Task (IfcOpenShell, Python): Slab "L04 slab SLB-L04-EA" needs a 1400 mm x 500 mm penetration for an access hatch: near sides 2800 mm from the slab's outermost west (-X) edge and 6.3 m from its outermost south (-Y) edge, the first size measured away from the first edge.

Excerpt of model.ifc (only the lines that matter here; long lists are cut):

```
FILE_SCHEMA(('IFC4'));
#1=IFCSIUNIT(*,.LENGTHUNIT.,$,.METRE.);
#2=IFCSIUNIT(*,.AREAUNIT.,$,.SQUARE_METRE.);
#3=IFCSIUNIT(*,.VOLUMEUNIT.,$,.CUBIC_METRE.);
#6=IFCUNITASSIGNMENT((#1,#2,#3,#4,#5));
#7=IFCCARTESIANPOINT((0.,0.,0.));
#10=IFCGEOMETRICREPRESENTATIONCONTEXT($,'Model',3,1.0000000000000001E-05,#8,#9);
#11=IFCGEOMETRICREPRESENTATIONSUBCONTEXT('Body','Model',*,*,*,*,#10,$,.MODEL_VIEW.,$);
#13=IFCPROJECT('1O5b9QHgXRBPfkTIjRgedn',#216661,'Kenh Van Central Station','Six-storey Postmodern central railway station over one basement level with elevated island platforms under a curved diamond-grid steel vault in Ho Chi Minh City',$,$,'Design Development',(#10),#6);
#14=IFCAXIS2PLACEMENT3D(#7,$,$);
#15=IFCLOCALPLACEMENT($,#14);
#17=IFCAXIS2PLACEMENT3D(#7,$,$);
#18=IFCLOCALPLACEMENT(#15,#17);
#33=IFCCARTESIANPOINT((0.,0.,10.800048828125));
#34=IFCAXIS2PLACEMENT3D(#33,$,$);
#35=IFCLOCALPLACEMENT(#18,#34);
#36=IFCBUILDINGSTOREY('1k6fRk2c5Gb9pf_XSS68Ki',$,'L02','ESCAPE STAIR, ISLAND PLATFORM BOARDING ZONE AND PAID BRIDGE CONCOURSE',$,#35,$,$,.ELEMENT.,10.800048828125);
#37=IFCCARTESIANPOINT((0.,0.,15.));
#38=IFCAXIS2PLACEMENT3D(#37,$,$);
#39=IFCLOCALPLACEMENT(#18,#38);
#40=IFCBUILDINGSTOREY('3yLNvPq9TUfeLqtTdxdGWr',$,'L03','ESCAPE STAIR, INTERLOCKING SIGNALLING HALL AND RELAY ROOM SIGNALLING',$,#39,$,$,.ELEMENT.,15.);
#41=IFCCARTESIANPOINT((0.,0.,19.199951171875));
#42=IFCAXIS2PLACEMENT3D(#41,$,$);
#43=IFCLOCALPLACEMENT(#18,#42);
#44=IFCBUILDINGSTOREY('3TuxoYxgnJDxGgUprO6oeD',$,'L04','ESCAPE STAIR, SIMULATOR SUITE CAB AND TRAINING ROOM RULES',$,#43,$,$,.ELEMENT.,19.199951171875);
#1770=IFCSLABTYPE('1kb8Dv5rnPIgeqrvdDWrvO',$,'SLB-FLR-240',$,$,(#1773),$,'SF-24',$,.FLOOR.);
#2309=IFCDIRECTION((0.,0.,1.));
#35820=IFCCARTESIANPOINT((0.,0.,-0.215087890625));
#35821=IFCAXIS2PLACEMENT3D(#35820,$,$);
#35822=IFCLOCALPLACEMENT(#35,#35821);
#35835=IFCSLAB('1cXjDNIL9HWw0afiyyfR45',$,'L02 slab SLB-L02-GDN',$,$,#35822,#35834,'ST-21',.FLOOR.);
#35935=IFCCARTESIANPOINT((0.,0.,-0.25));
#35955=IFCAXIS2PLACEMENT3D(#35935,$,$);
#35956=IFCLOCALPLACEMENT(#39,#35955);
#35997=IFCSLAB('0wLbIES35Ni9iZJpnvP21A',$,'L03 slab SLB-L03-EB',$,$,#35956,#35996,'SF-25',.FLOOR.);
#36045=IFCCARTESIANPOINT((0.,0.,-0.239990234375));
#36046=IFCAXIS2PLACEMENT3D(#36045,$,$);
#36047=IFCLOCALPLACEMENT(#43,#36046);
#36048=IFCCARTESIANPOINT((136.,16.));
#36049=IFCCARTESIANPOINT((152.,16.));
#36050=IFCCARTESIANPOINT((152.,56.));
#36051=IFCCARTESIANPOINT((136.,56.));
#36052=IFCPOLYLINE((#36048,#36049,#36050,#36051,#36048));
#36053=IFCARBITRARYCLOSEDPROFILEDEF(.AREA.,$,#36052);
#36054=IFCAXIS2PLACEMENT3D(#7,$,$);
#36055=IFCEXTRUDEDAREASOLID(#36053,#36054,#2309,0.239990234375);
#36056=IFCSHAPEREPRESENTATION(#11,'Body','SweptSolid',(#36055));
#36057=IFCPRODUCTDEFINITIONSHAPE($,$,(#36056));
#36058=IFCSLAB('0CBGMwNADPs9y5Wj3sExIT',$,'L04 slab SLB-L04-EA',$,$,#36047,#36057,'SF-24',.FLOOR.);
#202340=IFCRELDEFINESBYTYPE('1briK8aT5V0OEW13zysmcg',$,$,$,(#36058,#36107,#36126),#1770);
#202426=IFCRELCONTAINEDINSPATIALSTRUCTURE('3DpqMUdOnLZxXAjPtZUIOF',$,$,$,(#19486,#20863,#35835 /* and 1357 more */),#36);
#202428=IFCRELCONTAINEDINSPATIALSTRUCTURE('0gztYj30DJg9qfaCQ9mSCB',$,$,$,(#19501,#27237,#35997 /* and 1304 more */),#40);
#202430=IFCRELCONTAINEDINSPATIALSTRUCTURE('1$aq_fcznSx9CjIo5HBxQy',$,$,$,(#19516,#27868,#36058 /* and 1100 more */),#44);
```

```python
import numpy as np
import ifcopenshell
import ifcopenshell.api.feature
import ifcopenshell.api.geometry
import ifcopenshell.api.root
import ifcopenshell.geom
import ifcopenshell.util.placement
import ifcopenshell.util.representation
import ifcopenshell.util.shape
import ifcopenshell.util.unit

model = ifcopenshell.open("model.ifc")
unit_scale = ifcopenshell.util.unit.calculate_unit_scale(model)
settings = ifcopenshell.geom.settings()


def volume(element):
    """Net volume in cubic metres, openings subtracted."""
    shape = ifcopenshell.geom.create_shape(settings, element)
    return ifcopenshell.util.shape.get_volume(shape.geometry)


slab = model.by_guid("0CBGMwNADPs9y5Wj3sExIT")
before = volume(slab)

# Extent in the slab's own axes, in metres. The edges named are its -X and -Y sides.
slab_shape = ifcopenshell.geom.create_shape(settings, slab)
vertices = ifcopenshell.util.shape.get_vertices(slab_shape.geometry)
x_min, y_min, bottom = vertices.min(axis=0)
top = vertices[:, 2].max()

opening = ifcopenshell.api.root.create_entity(model, ifc_class="IfcOpeningElement", name="Access hatch opening", predefined_type="OPENING")
context = ifcopenshell.util.representation.get_context(model, "Model", "Body", "MODEL_VIEW")
width, depth = 1.4, 0.5
outline = [(0.0, 0.0), (width, 0.0), (width, depth), (0.0, depth), (0.0, 0.0)]
# Overshoot both faces by 50 mm so the cut is clean.
shape = ifcopenshell.api.geometry.add_slab_representation(
    model, context=context, depth=top - bottom + 0.1, polyline=outline
)
ifcopenshell.api.geometry.assign_representation(model, product=opening, representation=shape)

matrix = ifcopenshell.util.placement.get_local_placement(slab.ObjectPlacement)
matrix[:, 3] = matrix @ np.append(np.array([x_min + 2.8, y_min + 6.3, bottom - 0.05]) / unit_scale, 1.0)
ifcopenshell.api.geometry.edit_object_placement(model, product=opening, matrix=matrix, is_si=False)
ifcopenshell.api.feature.add_feature(model, feature=opening, element=slab)

after = volume(slab)

print(f"slab volume {before:.3f} -> {after:.3f} m3")

model.write("model-out.ifc")
```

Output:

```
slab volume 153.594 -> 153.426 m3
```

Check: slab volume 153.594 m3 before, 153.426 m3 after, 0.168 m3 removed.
